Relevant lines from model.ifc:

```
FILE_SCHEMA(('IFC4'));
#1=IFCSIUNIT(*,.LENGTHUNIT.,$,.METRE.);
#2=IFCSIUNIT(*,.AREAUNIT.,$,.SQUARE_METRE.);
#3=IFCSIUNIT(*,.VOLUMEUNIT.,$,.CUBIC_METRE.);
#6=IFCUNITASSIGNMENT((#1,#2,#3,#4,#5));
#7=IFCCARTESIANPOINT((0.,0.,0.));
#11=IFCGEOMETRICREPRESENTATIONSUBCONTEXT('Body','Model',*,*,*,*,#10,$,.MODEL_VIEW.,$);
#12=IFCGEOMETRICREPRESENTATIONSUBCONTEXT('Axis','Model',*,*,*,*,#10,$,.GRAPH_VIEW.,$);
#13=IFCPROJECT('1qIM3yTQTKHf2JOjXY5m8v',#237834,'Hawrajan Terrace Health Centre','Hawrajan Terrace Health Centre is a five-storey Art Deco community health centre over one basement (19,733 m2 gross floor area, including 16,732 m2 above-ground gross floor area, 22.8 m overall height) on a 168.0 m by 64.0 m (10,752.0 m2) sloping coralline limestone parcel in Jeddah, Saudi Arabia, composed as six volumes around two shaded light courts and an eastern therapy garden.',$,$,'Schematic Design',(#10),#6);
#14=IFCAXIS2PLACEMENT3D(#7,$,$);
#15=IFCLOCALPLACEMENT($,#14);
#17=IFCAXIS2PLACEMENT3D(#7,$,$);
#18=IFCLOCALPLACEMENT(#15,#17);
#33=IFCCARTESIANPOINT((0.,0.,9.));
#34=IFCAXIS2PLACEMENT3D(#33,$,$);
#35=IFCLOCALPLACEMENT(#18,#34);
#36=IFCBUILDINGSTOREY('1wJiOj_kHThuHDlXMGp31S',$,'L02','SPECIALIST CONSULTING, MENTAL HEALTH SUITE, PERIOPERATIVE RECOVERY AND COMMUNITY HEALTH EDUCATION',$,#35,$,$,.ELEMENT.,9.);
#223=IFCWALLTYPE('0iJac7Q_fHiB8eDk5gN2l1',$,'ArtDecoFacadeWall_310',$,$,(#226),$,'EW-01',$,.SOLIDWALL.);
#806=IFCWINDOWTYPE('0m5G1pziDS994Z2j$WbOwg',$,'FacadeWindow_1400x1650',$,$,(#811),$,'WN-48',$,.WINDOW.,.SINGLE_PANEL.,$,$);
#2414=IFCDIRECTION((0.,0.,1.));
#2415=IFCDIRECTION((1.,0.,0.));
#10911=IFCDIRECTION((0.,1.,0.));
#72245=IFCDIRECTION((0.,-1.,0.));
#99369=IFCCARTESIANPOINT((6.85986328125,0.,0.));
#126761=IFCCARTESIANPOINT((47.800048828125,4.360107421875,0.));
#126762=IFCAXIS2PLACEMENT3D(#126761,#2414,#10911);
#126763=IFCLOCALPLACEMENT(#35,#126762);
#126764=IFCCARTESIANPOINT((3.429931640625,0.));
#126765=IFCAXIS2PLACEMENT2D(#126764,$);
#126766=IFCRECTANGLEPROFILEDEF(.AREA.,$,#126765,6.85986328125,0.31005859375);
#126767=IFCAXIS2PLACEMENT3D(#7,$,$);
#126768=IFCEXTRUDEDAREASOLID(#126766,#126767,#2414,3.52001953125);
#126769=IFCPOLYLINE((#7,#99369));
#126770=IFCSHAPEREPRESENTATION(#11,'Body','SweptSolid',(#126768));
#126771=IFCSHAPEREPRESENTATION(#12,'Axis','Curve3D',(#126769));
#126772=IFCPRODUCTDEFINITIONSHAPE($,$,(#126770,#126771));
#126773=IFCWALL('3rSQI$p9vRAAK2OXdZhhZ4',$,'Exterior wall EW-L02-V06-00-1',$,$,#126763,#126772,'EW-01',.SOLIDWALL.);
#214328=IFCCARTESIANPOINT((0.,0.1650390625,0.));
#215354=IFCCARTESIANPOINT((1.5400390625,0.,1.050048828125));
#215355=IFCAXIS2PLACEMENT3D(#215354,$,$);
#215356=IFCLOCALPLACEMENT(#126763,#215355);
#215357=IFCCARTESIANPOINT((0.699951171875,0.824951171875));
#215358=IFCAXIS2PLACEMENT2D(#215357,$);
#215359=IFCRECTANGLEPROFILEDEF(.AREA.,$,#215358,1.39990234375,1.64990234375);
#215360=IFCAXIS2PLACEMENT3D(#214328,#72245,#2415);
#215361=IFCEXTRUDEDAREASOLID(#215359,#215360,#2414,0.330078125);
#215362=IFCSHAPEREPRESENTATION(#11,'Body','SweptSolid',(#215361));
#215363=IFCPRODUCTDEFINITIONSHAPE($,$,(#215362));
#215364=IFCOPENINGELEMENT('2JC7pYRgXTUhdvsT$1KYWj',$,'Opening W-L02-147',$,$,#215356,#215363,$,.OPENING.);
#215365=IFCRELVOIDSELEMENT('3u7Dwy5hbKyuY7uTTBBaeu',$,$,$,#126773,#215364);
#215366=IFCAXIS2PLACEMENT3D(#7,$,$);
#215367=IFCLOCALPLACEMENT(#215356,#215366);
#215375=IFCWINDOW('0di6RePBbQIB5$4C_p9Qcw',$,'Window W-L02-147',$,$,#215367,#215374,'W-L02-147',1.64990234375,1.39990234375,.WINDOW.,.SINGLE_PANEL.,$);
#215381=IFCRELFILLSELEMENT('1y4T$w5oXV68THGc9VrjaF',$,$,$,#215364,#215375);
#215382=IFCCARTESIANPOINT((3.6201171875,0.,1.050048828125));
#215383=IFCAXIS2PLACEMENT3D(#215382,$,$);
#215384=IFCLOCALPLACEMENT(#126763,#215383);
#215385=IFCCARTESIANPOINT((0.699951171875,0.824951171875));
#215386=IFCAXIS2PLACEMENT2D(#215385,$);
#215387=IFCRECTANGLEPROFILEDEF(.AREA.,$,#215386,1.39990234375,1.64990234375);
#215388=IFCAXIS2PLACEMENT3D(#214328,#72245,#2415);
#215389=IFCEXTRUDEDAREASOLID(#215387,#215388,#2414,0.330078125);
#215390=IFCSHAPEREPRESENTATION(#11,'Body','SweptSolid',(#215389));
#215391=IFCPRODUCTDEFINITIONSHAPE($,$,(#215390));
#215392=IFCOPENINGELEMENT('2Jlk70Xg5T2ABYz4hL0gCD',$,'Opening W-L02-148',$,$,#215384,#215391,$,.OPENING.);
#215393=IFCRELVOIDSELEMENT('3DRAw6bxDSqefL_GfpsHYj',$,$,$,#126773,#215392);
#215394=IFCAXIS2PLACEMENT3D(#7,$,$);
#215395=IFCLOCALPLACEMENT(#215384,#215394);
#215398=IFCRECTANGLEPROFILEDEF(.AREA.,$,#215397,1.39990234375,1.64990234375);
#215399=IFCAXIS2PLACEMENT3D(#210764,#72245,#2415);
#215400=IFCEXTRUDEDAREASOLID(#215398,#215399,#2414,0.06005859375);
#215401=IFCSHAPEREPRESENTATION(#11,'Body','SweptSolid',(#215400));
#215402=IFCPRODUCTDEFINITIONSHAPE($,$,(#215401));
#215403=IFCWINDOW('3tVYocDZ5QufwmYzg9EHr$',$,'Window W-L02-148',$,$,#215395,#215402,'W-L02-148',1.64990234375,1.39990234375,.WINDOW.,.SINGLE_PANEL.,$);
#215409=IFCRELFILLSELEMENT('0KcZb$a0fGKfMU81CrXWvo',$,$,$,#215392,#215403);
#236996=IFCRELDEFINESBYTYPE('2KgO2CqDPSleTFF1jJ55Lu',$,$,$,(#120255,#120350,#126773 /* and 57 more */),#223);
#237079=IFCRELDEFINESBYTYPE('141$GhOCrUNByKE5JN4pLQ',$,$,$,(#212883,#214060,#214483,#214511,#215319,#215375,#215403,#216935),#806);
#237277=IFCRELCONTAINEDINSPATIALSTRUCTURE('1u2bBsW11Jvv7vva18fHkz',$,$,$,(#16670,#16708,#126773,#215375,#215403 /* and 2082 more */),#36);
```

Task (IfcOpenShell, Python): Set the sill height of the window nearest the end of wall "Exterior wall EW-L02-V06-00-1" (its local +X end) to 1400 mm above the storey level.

```python
import numpy as np
import ifcopenshell
import ifcopenshell.api.geometry
import ifcopenshell.geom
import ifcopenshell.util.element
import ifcopenshell.util.placement
import ifcopenshell.util.shape
import ifcopenshell.util.unit

model = ifcopenshell.open("model.ifc")
unit_scale = ifcopenshell.util.unit.calculate_unit_scale(model)

window = model.by_guid("3tVYocDZ5QufwmYzg9EHr$")
opening = window.FillsVoids[0].RelatingOpeningElement
storey = ifcopenshell.util.element.get_container(window, ifc_class="IfcBuildingStorey")
level = ifcopenshell.util.placement.get_local_placement(storey.ObjectPlacement)[2, 3]

# The opening's origin need not be at the sill, so measure its lowest point.
shape = ifcopenshell.geom.create_shape(ifcopenshell.geom.settings(), opening)
bottom = ifcopenshell.util.shape.get_shape_bottom_elevation(shape, shape.geometry) / unit_scale
dz = level + 1.4 / unit_scale - bottom

shift = np.array([0.0, 0.0, dz])
# The window is placed relative to its opening, so it follows when the opening moves.
matrix = ifcopenshell.util.placement.get_local_placement(opening.ObjectPlacement)
matrix[:3, 3] += shift
ifcopenshell.api.geometry.edit_object_placement(
    model, product=opening, matrix=matrix, is_si=False, should_transform_children=True
)

print(f"moved by {dz * unit_scale:+.3f} m")

model.write("model_v2.ifc")
```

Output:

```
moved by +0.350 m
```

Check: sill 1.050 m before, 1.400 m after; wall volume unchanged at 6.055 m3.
